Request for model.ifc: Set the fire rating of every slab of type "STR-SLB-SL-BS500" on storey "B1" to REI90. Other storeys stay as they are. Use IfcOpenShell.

First a look at what the model holds.

```python
import ifcopenshell
import ifcopenshell.util.element

model = ifcopenshell.open("model.ifc")
print(model.schema)
storey = next(s for s in model.by_type("IfcBuildingStorey") if s.Name == "B1")
slabs = [e for e in ifcopenshell.util.element.get_decomposition(storey) if e.is_a("IfcSlab")]
seen = {}
for e in slabs:
    element_type = ifcopenshell.util.element.get_type(e)
    key = (element_type.Name if element_type != e and element_type else None, ifcopenshell.util.element.get_pset(e, "Pset_SlabCommon", "FireRating"))
    seen[key] = seen.get(key, 0) + 1
for (name, value), count in sorted(seen.items(), key=str):
    print(count, "x", name, "|", value)
```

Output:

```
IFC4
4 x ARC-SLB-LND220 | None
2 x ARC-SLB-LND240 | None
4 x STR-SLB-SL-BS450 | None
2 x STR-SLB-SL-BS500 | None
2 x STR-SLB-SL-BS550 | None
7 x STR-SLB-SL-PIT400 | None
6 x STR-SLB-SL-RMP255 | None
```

```python
import ifcopenshell
import ifcopenshell.api.pset
import ifcopenshell.util.element

model = ifcopenshell.open("model.ifc")

storey = next(s for s in model.by_type("IfcBuildingStorey") if s.Name == "B1")
slabs = [e for e in ifcopenshell.util.element.get_decomposition(storey) if e.is_a("IfcSlab")]

count = 0
for e in slabs:
    element_type = ifcopenshell.util.element.get_type(e)
    if element_type in (None, e) or element_type.Name != "STR-SLB-SL-BS500":
        continue
    # add_pset returns the element's existing set when there is one.
    pset = ifcopenshell.api.pset.add_pset(model, product=e, name="Pset_SlabCommon")
    ifcopenshell.api.pset.edit_pset(model, pset=pset, properties={"FireRating": "REI90"})
    count += 1

print(count, "slabs updated")

model.write("model_v2.ifc")
```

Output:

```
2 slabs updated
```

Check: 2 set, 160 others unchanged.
